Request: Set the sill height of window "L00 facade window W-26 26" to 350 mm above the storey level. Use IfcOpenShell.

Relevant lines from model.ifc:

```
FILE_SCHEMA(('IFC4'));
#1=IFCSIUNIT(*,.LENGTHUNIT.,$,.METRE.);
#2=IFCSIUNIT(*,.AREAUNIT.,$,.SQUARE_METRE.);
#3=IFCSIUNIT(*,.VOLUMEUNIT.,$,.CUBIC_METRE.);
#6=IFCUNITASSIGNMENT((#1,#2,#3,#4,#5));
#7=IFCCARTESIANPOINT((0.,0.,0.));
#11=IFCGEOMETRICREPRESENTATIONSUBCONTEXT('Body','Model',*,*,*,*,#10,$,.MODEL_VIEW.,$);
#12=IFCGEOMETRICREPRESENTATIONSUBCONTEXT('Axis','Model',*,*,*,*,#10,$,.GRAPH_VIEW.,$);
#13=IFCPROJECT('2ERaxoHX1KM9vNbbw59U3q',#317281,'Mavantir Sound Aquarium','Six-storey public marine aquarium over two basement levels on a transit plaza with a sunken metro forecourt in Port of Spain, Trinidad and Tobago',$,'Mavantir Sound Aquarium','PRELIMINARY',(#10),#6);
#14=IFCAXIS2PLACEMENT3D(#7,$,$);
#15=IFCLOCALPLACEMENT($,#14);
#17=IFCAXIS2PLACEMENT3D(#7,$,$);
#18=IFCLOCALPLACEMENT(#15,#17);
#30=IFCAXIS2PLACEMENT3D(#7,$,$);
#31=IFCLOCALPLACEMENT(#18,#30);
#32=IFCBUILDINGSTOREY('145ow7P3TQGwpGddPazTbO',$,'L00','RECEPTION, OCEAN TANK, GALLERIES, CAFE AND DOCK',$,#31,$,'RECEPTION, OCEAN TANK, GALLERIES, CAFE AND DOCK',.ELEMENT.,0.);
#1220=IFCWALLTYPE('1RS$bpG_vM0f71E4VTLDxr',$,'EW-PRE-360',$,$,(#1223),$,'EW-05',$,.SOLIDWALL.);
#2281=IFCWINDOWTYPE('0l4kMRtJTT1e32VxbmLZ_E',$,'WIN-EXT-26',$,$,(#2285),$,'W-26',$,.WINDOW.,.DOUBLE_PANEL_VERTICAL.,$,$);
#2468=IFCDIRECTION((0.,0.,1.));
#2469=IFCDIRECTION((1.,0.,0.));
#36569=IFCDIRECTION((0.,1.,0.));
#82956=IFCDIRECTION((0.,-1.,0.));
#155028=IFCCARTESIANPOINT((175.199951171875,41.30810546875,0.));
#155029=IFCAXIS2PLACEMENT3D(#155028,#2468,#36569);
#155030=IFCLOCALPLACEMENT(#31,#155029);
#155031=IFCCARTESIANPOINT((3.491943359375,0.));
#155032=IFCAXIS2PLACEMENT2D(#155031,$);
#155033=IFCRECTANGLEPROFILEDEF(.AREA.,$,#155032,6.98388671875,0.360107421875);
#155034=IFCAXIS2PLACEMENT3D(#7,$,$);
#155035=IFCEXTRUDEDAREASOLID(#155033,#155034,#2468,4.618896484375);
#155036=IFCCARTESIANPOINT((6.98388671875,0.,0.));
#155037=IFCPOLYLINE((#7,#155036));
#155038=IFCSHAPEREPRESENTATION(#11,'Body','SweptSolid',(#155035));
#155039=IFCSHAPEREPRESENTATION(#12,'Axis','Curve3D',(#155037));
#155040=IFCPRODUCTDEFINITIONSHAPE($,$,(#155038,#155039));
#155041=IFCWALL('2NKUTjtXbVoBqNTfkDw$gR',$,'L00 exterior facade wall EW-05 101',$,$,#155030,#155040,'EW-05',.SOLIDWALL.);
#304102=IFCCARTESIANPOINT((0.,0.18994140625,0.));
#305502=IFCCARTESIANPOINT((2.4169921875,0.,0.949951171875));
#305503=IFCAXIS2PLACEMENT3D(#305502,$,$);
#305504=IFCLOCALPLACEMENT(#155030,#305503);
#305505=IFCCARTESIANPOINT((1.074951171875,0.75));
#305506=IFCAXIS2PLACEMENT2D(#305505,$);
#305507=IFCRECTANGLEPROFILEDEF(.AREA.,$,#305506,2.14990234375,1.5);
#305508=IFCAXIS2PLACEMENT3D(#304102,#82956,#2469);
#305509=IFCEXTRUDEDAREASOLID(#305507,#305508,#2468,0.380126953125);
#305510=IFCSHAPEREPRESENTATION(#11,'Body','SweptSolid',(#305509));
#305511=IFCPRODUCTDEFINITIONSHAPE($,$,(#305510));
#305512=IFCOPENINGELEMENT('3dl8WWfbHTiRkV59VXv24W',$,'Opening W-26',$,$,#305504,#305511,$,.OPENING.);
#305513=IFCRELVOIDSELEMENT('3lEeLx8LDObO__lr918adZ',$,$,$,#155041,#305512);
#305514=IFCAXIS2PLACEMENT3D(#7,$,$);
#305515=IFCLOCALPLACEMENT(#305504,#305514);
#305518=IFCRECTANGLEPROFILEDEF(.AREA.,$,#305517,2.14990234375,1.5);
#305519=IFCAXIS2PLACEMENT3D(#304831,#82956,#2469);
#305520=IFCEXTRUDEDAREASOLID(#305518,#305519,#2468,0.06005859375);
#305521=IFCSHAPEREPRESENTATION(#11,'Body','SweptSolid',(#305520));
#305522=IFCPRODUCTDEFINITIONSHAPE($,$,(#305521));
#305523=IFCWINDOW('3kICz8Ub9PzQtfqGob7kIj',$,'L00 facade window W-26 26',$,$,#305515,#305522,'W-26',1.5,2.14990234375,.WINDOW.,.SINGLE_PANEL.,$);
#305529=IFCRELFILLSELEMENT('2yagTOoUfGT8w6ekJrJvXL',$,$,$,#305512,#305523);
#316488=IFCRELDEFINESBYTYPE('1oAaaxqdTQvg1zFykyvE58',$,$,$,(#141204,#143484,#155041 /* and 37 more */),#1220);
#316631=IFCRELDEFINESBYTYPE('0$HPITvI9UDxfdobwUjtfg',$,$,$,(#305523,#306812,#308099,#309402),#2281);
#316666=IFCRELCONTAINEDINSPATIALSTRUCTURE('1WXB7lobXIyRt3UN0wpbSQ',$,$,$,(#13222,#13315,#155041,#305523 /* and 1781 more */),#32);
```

```python
import numpy as np
import ifcopenshell
import ifcopenshell.api.geometry
import ifcopenshell.geom
import ifcopenshell.util.element
import ifcopenshell.util.placement
import ifcopenshell.util.shape
import ifcopenshell.util.unit

model = ifcopenshell.open("model.ifc")
unit_scale = ifcopenshell.util.unit.calculate_unit_scale(model)

window = model.by_guid("3kICz8Ub9PzQtfqGob7kIj")
opening = window.FillsVoids[0].RelatingOpeningElement
storey = ifcopenshell.util.element.get_container(window, ifc_class="IfcBuildingStorey")
level = ifcopenshell.util.placement.get_local_placement(storey.ObjectPlacement)[2, 3]

# The opening's origin need not be at the sill, so measure its lowest point.
shape = ifcopenshell.geom.create_shape(ifcopenshell.geom.settings(), opening)
bottom = ifcopenshell.util.shape.get_shape_bottom_elevation(shape, shape.geometry) / unit_scale
dz = level + 0.35 / unit_scale - bottom

shift = np.array([0.0, 0.0, dz])
# The window is placed relative to its opening, so it follows when the opening moves.
matrix = ifcopenshell.util.placement.get_local_placement(opening.ObjectPlacement)
matrix[:3, 3] += shift
ifcopenshell.api.geometry.edit_object_placement(
    model, product=opening, matrix=matrix, is_si=False, should_transform_children=True
)

print(f"moved by {dz * unit_scale:+.3f} m")

model.write("model_v2.ifc")
```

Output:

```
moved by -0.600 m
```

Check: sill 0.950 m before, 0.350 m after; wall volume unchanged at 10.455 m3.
